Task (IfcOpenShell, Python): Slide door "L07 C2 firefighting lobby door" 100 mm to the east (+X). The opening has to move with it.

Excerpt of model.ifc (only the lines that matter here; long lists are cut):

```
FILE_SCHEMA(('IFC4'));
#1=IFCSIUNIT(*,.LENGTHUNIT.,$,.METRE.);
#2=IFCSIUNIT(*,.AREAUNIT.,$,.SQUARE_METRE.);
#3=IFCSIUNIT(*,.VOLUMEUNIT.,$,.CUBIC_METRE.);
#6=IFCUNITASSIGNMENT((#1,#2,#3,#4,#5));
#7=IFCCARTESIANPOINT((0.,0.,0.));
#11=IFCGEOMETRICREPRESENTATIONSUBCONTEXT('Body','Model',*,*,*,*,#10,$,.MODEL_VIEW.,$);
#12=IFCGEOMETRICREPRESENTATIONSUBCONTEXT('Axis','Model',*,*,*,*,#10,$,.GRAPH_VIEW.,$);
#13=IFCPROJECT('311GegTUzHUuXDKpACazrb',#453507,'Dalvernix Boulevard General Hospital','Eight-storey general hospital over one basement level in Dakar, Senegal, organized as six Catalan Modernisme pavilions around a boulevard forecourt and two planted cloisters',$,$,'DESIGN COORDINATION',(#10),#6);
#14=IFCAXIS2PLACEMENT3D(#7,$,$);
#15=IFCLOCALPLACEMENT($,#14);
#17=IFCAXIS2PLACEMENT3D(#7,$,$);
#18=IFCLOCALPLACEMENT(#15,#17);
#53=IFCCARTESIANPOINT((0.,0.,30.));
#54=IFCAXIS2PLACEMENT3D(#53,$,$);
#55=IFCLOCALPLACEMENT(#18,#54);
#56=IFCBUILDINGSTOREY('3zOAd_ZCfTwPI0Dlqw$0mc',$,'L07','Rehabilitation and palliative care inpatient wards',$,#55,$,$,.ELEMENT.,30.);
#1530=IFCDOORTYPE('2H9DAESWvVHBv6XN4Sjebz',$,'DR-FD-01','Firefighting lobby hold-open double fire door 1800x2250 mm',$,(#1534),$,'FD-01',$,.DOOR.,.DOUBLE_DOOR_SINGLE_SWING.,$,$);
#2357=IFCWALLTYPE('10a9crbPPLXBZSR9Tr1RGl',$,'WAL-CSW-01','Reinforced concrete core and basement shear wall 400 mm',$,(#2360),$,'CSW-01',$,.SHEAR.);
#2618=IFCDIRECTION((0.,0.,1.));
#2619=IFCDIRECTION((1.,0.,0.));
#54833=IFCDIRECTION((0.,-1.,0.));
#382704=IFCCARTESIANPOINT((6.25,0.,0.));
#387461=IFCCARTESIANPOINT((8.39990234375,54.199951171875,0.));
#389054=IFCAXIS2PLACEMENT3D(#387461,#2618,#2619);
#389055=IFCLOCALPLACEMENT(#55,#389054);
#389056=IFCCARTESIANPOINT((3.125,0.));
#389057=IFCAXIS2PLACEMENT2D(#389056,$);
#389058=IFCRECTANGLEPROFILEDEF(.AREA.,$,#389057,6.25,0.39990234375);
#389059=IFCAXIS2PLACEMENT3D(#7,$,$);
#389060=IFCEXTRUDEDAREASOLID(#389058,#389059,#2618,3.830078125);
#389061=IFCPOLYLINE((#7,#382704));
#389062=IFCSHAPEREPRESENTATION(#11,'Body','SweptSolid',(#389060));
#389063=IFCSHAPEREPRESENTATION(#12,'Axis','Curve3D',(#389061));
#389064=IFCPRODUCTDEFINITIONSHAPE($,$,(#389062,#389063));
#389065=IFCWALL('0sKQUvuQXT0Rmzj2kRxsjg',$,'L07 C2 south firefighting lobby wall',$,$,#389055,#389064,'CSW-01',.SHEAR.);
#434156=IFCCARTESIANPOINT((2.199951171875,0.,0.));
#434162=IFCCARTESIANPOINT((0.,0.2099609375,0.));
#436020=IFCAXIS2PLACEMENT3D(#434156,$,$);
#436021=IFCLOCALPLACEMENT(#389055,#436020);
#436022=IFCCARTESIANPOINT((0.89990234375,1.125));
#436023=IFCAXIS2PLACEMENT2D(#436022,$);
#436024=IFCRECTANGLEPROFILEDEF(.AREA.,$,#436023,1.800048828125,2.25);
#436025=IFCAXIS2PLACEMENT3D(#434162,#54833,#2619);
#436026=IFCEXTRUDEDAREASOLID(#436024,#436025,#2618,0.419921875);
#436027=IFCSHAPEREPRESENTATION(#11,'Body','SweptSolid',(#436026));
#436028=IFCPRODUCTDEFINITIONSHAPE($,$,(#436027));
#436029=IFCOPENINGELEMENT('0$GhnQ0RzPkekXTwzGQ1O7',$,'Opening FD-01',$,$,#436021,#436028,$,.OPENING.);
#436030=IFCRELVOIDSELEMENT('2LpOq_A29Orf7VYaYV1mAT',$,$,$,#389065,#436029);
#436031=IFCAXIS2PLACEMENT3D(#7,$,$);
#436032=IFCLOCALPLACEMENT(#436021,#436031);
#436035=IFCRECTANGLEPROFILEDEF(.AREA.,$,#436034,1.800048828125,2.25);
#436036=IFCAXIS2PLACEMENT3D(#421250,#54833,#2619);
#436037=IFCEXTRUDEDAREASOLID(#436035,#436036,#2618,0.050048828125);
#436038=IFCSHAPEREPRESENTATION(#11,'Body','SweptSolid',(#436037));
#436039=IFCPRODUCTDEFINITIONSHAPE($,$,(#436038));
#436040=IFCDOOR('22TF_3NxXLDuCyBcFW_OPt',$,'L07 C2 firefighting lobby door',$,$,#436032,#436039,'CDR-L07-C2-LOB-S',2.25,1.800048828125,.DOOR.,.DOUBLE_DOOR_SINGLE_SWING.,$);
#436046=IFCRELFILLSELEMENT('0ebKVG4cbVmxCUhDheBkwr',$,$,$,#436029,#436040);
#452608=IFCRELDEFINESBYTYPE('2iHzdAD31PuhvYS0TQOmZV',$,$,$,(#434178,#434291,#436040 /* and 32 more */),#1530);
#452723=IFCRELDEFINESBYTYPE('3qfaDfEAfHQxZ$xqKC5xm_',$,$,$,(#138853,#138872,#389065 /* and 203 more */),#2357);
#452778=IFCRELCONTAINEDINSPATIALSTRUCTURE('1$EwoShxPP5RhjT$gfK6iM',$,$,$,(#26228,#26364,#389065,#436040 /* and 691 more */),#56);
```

```python
import ifcopenshell
import ifcopenshell.api.geometry
import ifcopenshell.util.placement

model = ifcopenshell.open("model.ifc")

door = model.by_guid("22TF_3NxXLDuCyBcFW_OPt")
opening = door.FillsVoids[0].RelatingOpeningElement
wall = opening.VoidsElements[0].RelatingBuildingElement

wall_matrix = ifcopenshell.util.placement.get_local_placement(wall.ObjectPlacement)
shift = wall_matrix[:3, 0] * 0.1
before = ifcopenshell.util.placement.get_local_placement(door.ObjectPlacement)[:3, 3].copy()

# The door is placed relative to its opening, so it follows when the opening moves.
matrix = ifcopenshell.util.placement.get_local_placement(opening.ObjectPlacement)
matrix[:3, 3] += shift
ifcopenshell.api.geometry.edit_object_placement(
    model, product=opening, matrix=matrix, is_si=False, should_transform_children=True
)

after = ifcopenshell.util.placement.get_local_placement(door.ObjectPlacement)[:3, 3]
print("door moved by", (after - before).round(3) + 0.0)

model.write("model-out.ifc")
```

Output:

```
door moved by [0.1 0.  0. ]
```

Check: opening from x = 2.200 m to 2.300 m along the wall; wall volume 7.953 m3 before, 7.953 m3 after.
